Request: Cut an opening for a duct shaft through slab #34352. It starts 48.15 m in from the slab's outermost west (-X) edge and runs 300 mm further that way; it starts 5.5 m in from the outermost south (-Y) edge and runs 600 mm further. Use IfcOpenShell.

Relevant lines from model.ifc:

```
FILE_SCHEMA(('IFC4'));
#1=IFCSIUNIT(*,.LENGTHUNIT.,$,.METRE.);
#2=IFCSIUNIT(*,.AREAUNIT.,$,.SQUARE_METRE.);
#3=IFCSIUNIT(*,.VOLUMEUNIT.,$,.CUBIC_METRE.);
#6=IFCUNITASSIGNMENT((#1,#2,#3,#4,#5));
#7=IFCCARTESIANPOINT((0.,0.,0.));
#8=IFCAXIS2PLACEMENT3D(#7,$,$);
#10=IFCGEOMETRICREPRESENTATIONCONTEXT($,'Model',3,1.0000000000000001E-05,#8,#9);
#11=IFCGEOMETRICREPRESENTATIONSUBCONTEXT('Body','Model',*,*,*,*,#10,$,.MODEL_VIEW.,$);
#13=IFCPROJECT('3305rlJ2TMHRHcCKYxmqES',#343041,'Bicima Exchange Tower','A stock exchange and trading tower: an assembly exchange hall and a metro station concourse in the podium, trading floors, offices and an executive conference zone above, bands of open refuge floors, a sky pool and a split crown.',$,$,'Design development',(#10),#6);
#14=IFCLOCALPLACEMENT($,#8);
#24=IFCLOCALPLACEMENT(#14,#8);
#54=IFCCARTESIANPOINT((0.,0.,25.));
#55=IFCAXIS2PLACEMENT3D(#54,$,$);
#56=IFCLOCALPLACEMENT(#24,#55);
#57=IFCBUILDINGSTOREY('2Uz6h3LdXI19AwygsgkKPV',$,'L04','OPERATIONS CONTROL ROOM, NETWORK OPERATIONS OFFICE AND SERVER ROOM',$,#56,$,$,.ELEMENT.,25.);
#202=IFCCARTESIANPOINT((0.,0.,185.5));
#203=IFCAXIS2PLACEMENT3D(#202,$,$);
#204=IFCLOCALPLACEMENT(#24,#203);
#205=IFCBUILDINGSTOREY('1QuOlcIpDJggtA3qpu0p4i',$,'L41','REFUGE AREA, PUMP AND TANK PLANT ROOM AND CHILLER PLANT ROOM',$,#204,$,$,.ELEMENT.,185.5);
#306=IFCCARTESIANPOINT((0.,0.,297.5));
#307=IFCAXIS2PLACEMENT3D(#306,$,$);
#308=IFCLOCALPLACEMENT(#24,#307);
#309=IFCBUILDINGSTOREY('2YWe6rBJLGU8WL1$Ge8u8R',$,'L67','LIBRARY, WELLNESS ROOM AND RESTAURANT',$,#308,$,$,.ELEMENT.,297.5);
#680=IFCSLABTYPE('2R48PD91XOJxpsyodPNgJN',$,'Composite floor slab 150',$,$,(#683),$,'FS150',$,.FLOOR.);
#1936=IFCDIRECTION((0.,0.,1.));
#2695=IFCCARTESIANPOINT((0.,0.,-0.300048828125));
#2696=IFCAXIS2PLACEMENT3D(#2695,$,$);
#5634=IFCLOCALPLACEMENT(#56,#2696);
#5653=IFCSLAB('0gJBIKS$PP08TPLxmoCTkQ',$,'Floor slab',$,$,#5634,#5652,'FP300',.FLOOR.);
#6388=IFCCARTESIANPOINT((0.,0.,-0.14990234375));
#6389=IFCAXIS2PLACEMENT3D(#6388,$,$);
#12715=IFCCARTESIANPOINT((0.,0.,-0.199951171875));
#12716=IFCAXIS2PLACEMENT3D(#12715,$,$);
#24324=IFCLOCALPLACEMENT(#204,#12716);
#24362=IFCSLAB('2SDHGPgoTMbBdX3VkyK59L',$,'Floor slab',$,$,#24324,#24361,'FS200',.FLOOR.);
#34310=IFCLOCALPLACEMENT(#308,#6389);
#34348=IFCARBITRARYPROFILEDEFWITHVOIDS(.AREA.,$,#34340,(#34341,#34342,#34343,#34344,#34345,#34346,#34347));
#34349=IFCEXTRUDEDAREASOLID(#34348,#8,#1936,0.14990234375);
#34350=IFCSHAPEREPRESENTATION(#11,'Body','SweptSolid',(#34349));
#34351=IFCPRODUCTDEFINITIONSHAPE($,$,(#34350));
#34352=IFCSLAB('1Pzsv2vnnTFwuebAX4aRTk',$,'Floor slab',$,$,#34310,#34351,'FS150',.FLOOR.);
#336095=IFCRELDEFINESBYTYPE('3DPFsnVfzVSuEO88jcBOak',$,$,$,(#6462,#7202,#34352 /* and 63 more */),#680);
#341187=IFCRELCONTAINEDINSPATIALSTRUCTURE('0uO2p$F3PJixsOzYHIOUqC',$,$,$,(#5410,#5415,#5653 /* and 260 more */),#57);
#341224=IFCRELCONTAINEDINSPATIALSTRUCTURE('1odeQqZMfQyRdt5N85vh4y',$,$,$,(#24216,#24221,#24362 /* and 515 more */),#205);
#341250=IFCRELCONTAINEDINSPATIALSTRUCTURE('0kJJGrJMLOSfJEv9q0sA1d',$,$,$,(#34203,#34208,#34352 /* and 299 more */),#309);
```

```python
import numpy as np
import ifcopenshell
import ifcopenshell.api.feature
import ifcopenshell.api.geometry
import ifcopenshell.api.root
import ifcopenshell.geom
import ifcopenshell.util.placement
import ifcopenshell.util.representation
import ifcopenshell.util.shape
import ifcopenshell.util.unit

model = ifcopenshell.open("model.ifc")
unit_scale = ifcopenshell.util.unit.calculate_unit_scale(model)
settings = ifcopenshell.geom.settings()


def volume(element):
    """Net volume in cubic metres, openings subtracted."""
    shape = ifcopenshell.geom.create_shape(settings, element)
    return ifcopenshell.util.shape.get_volume(shape.geometry)


slab = model.by_id(34352)
before = volume(slab)

# Extent in the slab's own axes, in metres. The edges named are its -X and -Y sides.
slab_shape = ifcopenshell.geom.create_shape(settings, slab)
vertices = ifcopenshell.util.shape.get_vertices(slab_shape.geometry)
x_min, y_min, bottom = vertices.min(axis=0)
top = vertices[:, 2].max()

opening = ifcopenshell.api.root.create_entity(model, ifc_class="IfcOpeningElement", name="Duct shaft opening", predefined_type="OPENING")
context = ifcopenshell.util.representation.get_context(model, "Model", "Body", "MODEL_VIEW")
width, depth = 0.3, 0.6
outline = [(0.0, 0.0), (width, 0.0), (width, depth), (0.0, depth), (0.0, 0.0)]
# Overshoot both faces by 50 mm so the cut is clean.
shape = ifcopenshell.api.geometry.add_slab_representation(
    model, context=context, depth=top - bottom + 0.1, polyline=outline
)
ifcopenshell.api.geometry.assign_representation(model, product=opening, representation=shape)

matrix = ifcopenshell.util.placement.get_local_placement(slab.ObjectPlacement)
matrix[:, 3] = matrix @ np.append(np.array([x_min + 48.15, y_min + 5.5, bottom - 0.05]) / unit_scale, 1.0)
ifcopenshell.api.geometry.edit_object_placement(model, product=opening, matrix=matrix, is_si=False)
ifcopenshell.api.feature.add_feature(model, feature=opening, element=slab)

after = volume(slab)

print(f"slab volume {before:.3f} -> {after:.3f} m3")

model.write("model_edited.ifc")
```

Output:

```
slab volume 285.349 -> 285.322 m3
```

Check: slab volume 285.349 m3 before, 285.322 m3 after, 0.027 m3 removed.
